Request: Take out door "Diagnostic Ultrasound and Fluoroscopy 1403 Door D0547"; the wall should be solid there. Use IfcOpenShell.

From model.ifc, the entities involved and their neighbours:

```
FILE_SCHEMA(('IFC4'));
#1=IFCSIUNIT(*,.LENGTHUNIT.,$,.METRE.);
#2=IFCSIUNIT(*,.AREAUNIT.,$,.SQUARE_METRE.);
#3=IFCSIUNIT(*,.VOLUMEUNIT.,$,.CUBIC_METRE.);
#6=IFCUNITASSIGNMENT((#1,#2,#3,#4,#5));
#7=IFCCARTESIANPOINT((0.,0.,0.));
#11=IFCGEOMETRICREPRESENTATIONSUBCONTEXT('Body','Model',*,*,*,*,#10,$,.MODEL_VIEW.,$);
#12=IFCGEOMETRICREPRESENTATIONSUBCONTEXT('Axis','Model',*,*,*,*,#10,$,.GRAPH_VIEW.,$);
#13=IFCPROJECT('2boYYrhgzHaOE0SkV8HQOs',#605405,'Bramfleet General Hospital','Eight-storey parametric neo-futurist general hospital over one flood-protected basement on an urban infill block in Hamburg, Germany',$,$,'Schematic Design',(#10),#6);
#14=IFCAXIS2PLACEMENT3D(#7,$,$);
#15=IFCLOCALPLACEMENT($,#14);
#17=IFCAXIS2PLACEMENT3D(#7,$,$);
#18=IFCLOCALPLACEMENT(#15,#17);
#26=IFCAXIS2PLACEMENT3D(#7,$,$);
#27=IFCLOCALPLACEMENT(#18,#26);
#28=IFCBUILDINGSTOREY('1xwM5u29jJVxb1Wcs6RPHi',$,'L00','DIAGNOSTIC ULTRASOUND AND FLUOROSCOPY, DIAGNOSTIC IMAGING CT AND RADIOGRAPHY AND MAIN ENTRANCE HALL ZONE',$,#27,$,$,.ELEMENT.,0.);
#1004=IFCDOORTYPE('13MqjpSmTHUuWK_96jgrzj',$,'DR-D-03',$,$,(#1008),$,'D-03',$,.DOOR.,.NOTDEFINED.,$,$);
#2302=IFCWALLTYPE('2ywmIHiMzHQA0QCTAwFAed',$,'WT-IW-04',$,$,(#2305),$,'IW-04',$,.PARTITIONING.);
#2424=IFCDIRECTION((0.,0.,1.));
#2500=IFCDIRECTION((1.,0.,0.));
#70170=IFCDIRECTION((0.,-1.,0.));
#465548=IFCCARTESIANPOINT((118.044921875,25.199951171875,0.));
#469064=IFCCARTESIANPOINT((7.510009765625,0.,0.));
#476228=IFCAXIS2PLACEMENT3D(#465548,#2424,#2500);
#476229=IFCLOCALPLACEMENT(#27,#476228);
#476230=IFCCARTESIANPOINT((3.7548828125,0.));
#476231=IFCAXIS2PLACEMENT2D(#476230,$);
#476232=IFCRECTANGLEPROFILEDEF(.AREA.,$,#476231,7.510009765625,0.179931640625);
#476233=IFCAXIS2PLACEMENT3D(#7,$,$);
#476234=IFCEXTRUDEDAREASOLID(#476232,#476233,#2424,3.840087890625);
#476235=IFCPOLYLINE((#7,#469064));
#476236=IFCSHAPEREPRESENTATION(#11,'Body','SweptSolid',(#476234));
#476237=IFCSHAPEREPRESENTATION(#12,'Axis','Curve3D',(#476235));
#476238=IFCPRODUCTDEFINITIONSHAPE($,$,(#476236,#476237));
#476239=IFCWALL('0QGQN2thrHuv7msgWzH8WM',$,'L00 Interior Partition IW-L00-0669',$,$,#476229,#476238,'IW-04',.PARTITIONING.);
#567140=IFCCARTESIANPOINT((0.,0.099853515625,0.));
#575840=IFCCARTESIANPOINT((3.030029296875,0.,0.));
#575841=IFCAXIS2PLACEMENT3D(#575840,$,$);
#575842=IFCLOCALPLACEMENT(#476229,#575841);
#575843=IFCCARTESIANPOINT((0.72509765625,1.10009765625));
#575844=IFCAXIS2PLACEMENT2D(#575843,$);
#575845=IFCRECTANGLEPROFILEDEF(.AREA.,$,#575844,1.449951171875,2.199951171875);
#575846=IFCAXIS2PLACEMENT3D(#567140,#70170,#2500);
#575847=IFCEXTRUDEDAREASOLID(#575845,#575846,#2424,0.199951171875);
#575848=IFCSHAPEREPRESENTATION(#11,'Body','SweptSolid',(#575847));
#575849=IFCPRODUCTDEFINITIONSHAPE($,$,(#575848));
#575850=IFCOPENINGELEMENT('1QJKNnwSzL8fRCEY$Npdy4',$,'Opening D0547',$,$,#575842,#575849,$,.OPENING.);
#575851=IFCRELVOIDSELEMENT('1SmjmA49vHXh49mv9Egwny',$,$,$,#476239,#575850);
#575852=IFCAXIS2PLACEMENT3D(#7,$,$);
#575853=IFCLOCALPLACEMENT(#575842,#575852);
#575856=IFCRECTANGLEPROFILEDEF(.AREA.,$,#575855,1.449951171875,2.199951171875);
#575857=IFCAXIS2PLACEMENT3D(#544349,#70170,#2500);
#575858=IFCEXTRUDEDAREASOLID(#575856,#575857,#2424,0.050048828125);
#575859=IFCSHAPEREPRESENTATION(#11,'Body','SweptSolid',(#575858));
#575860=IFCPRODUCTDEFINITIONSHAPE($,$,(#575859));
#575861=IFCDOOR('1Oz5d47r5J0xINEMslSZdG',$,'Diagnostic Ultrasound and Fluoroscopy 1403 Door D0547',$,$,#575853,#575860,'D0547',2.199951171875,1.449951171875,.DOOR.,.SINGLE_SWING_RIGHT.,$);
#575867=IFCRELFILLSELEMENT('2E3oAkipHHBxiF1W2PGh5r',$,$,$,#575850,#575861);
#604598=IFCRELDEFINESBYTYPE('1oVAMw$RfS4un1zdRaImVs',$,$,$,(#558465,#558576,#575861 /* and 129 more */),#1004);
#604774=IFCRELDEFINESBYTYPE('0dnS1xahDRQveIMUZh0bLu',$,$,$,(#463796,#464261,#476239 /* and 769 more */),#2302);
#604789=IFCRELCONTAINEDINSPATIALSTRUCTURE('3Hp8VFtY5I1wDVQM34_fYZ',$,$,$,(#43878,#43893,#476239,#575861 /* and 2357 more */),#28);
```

```python
import ifcopenshell
import ifcopenshell.api.feature
import ifcopenshell.api.root
import ifcopenshell.geom
import ifcopenshell.util.shape

model = ifcopenshell.open("model.ifc")
settings = ifcopenshell.geom.settings()


def volume(element):
    """Net volume in cubic metres, openings subtracted."""
    shape = ifcopenshell.geom.create_shape(settings, element)
    return ifcopenshell.util.shape.get_volume(shape.geometry)


door = model.by_guid("1Oz5d47r5J0xINEMslSZdG")
opening = door.FillsVoids[0].RelatingOpeningElement
wall = opening.VoidsElements[0].RelatingBuildingElement
before = volume(wall)

ifcopenshell.api.root.remove_product(model, product=door)
ifcopenshell.api.feature.remove_feature(model, feature=opening)

after = volume(wall)

print(f"wall volume {before:.3f} -> {after:.3f} m3")

model.write("model_rev.ifc")
```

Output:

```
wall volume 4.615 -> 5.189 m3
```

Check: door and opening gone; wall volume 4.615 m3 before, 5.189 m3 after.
